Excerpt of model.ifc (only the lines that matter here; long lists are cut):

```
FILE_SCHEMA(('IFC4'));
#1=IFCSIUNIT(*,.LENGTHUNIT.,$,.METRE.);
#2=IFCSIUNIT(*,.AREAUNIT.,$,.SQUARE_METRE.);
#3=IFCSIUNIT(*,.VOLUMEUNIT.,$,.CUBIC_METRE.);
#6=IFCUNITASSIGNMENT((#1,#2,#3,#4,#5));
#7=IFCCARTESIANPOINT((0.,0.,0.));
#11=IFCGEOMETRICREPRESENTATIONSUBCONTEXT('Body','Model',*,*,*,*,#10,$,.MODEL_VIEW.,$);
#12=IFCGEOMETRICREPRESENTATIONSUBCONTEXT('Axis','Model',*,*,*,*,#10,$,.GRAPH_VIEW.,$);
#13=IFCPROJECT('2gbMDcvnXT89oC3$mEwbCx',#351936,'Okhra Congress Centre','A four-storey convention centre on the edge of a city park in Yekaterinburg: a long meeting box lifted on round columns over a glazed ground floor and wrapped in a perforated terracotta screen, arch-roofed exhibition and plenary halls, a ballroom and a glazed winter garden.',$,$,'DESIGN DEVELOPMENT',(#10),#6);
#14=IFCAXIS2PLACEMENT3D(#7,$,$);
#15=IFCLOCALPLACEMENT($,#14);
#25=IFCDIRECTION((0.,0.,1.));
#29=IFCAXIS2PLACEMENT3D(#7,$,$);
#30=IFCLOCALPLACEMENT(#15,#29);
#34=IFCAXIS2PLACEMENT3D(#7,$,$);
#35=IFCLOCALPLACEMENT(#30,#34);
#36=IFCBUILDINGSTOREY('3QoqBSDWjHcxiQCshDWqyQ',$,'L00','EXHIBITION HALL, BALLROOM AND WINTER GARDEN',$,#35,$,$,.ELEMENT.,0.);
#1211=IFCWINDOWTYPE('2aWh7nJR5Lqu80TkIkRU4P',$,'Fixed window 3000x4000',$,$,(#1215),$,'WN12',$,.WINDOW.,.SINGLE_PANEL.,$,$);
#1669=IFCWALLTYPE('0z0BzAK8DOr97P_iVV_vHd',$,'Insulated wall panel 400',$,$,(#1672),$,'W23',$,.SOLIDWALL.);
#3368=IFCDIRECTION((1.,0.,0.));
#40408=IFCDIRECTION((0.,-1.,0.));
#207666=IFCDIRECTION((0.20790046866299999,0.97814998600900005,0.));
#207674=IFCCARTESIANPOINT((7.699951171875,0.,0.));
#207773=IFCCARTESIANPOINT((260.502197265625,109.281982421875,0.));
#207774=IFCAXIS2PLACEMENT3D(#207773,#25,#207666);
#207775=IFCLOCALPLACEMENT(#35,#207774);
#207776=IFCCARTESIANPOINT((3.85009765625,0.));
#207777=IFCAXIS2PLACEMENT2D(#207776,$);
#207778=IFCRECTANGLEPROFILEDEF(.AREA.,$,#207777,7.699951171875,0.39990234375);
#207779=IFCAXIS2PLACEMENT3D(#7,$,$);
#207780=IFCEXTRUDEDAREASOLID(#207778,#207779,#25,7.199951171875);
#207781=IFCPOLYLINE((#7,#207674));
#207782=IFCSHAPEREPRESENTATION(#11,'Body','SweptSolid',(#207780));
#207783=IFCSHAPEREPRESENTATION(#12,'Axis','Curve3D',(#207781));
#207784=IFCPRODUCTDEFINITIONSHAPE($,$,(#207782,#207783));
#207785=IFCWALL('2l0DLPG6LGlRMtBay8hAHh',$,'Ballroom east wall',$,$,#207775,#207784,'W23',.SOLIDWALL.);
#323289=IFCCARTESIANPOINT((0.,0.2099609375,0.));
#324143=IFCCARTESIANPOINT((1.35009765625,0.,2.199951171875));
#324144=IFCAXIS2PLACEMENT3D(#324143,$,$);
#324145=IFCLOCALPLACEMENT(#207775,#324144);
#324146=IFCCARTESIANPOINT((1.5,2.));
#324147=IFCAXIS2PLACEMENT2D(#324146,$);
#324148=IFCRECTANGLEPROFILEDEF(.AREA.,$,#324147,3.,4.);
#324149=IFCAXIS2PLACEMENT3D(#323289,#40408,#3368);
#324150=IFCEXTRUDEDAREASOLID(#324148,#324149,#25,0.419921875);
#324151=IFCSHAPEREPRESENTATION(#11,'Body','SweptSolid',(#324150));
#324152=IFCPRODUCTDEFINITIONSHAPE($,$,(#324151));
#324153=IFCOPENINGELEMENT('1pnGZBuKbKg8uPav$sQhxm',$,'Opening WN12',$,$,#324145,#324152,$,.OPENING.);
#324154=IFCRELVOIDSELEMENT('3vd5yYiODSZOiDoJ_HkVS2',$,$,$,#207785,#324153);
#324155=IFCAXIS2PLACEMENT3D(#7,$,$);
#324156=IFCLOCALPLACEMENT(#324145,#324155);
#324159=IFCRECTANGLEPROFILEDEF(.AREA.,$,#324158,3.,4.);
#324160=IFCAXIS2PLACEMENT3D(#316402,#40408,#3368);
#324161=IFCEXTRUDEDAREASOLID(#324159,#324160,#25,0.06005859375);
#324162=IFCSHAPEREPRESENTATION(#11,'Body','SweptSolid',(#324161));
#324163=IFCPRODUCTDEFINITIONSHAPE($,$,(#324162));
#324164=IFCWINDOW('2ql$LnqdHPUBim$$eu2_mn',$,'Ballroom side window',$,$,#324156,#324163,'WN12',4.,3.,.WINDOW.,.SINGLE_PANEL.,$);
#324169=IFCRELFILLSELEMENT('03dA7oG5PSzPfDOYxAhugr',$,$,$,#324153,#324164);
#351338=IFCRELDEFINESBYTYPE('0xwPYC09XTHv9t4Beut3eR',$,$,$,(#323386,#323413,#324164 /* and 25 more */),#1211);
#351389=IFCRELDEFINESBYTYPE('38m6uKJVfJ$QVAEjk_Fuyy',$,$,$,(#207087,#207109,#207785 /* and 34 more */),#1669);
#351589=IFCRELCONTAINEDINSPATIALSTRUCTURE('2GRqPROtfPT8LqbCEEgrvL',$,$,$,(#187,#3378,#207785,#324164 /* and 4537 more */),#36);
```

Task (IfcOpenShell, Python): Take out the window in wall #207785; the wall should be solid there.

```python
import ifcopenshell
import ifcopenshell.api.feature
import ifcopenshell.api.root
import ifcopenshell.geom
import ifcopenshell.util.shape

model = ifcopenshell.open("model.ifc")
settings = ifcopenshell.geom.settings()


def volume(element):
    """Net volume in cubic metres, openings subtracted."""
    shape = ifcopenshell.geom.create_shape(settings, element)
    return ifcopenshell.util.shape.get_volume(shape.geometry)


window = model.by_guid("2ql$LnqdHPUBim$$eu2_mn")
opening = window.FillsVoids[0].RelatingOpeningElement
wall = opening.VoidsElements[0].RelatingBuildingElement
before = volume(wall)

ifcopenshell.api.root.remove_product(model, product=window)
ifcopenshell.api.feature.remove_feature(model, feature=opening)

after = volume(wall)

print(f"wall volume {before:.3f} -> {after:.3f} m3")

model.write("model_rev.ifc")
```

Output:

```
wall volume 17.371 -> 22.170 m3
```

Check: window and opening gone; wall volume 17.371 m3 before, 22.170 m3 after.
